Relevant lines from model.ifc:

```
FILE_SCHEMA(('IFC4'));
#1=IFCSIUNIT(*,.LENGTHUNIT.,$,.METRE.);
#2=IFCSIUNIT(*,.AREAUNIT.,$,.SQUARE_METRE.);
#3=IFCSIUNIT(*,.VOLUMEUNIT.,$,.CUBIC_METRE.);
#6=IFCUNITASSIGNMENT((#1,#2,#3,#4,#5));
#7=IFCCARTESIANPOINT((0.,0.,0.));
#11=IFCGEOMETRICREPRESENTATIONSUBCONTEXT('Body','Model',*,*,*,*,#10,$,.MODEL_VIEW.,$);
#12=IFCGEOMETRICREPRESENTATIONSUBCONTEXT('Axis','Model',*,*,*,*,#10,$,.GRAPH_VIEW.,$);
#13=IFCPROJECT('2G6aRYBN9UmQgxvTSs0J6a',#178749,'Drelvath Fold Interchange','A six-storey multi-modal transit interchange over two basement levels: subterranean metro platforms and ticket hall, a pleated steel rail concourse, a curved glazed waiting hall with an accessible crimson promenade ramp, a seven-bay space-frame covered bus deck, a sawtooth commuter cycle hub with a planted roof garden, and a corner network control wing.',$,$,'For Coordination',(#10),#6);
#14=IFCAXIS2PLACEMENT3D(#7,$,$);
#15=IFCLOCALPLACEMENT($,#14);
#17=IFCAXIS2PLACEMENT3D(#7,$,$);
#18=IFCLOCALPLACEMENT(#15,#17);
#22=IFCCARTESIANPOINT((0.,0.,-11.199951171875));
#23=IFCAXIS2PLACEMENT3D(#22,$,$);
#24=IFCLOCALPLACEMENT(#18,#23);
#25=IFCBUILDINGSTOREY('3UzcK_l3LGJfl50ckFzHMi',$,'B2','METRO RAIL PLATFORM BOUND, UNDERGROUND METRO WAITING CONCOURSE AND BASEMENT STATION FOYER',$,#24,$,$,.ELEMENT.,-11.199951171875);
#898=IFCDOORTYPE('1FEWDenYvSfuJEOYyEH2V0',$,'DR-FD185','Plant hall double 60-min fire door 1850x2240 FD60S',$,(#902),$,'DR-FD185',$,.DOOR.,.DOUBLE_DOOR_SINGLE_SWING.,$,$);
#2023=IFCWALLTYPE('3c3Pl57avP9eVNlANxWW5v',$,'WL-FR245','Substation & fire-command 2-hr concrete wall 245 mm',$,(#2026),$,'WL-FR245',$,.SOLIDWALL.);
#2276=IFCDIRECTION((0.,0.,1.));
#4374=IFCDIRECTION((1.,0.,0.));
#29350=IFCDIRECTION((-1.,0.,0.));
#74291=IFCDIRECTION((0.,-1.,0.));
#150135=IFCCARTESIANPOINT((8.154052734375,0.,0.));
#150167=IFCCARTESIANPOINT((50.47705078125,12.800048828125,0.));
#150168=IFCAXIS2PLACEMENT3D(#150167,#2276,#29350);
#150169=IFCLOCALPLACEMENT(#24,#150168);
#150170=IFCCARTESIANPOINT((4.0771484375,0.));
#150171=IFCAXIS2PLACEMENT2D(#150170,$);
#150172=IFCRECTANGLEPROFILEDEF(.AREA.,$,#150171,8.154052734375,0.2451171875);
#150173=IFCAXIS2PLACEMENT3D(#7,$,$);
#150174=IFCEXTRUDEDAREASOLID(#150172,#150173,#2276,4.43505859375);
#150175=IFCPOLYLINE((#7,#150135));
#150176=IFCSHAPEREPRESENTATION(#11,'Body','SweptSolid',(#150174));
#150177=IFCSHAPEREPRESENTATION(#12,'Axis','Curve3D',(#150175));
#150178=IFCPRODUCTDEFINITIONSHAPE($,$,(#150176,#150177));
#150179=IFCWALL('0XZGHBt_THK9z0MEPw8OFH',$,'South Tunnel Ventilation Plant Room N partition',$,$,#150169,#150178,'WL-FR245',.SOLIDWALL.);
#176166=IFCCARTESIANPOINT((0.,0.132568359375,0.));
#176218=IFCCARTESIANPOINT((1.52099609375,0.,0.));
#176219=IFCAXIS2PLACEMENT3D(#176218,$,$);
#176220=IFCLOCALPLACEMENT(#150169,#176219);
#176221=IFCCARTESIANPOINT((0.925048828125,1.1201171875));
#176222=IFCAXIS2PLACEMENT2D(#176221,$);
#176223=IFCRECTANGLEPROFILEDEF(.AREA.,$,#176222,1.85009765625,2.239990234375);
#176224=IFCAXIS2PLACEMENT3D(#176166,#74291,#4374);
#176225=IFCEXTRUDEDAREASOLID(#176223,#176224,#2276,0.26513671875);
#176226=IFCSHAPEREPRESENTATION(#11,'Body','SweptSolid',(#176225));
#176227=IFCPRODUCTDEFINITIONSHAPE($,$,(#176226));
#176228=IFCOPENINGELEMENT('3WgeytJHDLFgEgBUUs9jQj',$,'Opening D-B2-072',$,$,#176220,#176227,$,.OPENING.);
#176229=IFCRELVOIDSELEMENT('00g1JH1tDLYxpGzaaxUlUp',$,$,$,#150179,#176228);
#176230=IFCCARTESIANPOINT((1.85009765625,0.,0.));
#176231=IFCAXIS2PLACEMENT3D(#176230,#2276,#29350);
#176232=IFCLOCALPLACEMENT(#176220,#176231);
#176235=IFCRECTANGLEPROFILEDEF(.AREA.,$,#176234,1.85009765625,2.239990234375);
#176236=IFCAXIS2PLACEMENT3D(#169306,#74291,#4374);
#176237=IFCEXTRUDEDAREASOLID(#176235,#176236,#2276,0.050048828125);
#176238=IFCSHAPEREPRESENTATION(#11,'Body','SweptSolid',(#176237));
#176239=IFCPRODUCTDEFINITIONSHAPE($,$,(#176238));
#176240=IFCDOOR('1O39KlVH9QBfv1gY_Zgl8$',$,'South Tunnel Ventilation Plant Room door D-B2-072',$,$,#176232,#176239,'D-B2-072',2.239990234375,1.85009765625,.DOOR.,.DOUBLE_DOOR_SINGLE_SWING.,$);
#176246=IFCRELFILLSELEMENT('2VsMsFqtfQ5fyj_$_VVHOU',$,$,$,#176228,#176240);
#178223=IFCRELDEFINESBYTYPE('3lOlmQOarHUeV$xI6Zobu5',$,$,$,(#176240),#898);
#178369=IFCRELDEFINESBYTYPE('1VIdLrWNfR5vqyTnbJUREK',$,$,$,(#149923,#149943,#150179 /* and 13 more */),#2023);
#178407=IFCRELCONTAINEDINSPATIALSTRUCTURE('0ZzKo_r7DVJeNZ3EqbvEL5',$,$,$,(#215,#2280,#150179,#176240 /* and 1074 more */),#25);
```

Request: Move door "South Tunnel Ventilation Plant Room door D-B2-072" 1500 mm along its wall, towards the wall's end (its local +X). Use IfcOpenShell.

```python
import ifcopenshell
import ifcopenshell.api.geometry
import ifcopenshell.util.placement
import ifcopenshell.util.unit

model = ifcopenshell.open("model.ifc")
unit_scale = ifcopenshell.util.unit.calculate_unit_scale(model)

door = model.by_id(176240)
opening = door.FillsVoids[0].RelatingOpeningElement
wall = opening.VoidsElements[0].RelatingBuildingElement

wall_matrix = ifcopenshell.util.placement.get_local_placement(wall.ObjectPlacement)
shift = wall_matrix[:3, 0] * 1.5 / unit_scale
before = ifcopenshell.util.placement.get_local_placement(door.ObjectPlacement)[:3, 3].copy()

# The door is placed relative to its opening, so it follows when the opening moves.
matrix = ifcopenshell.util.placement.get_local_placement(opening.ObjectPlacement)
matrix[:3, 3] += shift
ifcopenshell.api.geometry.edit_object_placement(
    model, product=opening, matrix=matrix, is_si=False, should_transform_children=True
)

after = ifcopenshell.util.placement.get_local_placement(door.ObjectPlacement)[:3, 3]
print("door moved by", (after - before).round(3) + 0.0)

model.write("model-out.ifc")
```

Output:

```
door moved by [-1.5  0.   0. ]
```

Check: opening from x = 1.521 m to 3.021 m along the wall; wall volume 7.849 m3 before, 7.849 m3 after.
